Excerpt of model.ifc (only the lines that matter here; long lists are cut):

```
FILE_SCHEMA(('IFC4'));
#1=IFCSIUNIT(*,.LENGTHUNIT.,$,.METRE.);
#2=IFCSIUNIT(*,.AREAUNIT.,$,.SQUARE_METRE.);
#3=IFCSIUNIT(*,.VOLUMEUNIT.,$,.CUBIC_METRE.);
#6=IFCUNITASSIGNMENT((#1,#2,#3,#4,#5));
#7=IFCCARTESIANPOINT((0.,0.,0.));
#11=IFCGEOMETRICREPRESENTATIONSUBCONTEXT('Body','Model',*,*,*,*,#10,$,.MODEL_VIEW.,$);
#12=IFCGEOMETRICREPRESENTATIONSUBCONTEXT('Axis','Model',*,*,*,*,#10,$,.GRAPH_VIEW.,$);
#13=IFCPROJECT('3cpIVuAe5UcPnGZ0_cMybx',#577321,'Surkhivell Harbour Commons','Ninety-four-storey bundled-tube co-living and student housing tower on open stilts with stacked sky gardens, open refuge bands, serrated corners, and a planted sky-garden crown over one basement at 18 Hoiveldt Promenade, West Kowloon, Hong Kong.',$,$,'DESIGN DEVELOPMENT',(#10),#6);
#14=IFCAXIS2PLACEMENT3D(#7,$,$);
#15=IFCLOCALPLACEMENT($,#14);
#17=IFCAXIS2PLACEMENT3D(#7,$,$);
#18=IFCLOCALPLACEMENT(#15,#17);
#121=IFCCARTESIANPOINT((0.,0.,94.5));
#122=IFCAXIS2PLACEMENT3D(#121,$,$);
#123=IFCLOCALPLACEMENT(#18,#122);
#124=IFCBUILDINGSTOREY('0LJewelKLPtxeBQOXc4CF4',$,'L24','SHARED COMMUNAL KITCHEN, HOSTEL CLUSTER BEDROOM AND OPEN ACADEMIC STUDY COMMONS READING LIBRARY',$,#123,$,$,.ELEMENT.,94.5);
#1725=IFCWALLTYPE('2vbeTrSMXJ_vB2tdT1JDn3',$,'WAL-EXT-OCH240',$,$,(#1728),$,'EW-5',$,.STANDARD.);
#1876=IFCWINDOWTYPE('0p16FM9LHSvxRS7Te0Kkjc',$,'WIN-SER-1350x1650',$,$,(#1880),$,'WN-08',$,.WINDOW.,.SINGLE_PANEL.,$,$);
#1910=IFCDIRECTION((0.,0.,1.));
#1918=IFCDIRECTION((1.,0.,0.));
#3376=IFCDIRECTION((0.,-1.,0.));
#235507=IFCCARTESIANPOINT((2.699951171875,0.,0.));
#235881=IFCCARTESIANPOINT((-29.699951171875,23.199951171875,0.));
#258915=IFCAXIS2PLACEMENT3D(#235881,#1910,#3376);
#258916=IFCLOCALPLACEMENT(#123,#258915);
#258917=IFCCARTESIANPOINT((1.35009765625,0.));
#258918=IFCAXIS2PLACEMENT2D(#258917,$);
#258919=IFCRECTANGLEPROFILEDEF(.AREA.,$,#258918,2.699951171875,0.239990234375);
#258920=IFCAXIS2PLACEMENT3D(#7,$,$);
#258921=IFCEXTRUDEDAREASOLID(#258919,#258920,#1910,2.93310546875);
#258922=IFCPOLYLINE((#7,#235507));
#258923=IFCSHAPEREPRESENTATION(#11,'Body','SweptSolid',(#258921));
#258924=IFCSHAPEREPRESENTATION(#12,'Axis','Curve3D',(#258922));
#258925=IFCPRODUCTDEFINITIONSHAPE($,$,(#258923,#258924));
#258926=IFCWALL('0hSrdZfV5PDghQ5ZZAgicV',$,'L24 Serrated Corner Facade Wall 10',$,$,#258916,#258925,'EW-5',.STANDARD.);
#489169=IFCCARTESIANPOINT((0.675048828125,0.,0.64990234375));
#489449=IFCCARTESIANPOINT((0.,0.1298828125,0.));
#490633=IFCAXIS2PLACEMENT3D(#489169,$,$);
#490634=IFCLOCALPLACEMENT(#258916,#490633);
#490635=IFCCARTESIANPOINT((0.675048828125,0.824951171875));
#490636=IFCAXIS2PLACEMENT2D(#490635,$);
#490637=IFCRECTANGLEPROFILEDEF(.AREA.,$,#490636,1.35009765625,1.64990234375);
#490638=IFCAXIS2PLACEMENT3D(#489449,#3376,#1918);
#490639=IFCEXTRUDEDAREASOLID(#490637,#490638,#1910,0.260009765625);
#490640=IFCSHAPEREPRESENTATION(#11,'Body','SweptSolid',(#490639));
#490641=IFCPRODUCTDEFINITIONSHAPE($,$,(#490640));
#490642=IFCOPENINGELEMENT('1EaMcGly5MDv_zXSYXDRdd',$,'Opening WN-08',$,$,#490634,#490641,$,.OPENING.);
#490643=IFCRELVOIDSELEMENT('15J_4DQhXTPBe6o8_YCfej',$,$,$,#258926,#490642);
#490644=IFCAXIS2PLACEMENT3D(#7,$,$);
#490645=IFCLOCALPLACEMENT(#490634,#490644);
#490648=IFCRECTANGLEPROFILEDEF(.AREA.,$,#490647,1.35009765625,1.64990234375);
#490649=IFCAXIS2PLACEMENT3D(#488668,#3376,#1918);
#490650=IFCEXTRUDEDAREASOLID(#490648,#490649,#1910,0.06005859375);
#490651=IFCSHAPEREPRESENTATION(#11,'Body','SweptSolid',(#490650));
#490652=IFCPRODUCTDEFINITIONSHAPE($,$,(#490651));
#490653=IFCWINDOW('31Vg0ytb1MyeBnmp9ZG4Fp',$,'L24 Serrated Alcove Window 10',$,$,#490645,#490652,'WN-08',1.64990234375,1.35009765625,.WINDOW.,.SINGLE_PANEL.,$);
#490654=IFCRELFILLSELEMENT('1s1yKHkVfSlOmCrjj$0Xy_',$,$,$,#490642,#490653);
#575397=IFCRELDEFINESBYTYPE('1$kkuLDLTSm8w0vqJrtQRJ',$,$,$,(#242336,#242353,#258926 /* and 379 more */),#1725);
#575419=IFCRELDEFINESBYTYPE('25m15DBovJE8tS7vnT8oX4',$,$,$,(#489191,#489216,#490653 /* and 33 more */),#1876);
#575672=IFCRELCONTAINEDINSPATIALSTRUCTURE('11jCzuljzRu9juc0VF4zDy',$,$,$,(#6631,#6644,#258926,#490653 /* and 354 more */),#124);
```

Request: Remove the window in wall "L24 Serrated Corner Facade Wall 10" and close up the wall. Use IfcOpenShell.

```python
import ifcopenshell
import ifcopenshell.api.feature
import ifcopenshell.api.root
import ifcopenshell.geom
import ifcopenshell.util.shape

model = ifcopenshell.open("model.ifc")
settings = ifcopenshell.geom.settings()


def volume(element):
    """Net volume in cubic metres, openings subtracted."""
    shape = ifcopenshell.geom.create_shape(settings, element)
    return ifcopenshell.util.shape.get_volume(shape.geometry)


window = model.by_guid("31Vg0ytb1MyeBnmp9ZG4Fp")
opening = window.FillsVoids[0].RelatingOpeningElement
wall = opening.VoidsElements[0].RelatingBuildingElement
before = volume(wall)

ifcopenshell.api.root.remove_product(model, product=window)
ifcopenshell.api.feature.remove_feature(model, feature=opening)

after = volume(wall)

print(f"wall volume {before:.3f} -> {after:.3f} m3")

model.write("model_v2.ifc")
```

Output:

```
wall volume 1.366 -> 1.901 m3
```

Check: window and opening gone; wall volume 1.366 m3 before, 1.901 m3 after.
